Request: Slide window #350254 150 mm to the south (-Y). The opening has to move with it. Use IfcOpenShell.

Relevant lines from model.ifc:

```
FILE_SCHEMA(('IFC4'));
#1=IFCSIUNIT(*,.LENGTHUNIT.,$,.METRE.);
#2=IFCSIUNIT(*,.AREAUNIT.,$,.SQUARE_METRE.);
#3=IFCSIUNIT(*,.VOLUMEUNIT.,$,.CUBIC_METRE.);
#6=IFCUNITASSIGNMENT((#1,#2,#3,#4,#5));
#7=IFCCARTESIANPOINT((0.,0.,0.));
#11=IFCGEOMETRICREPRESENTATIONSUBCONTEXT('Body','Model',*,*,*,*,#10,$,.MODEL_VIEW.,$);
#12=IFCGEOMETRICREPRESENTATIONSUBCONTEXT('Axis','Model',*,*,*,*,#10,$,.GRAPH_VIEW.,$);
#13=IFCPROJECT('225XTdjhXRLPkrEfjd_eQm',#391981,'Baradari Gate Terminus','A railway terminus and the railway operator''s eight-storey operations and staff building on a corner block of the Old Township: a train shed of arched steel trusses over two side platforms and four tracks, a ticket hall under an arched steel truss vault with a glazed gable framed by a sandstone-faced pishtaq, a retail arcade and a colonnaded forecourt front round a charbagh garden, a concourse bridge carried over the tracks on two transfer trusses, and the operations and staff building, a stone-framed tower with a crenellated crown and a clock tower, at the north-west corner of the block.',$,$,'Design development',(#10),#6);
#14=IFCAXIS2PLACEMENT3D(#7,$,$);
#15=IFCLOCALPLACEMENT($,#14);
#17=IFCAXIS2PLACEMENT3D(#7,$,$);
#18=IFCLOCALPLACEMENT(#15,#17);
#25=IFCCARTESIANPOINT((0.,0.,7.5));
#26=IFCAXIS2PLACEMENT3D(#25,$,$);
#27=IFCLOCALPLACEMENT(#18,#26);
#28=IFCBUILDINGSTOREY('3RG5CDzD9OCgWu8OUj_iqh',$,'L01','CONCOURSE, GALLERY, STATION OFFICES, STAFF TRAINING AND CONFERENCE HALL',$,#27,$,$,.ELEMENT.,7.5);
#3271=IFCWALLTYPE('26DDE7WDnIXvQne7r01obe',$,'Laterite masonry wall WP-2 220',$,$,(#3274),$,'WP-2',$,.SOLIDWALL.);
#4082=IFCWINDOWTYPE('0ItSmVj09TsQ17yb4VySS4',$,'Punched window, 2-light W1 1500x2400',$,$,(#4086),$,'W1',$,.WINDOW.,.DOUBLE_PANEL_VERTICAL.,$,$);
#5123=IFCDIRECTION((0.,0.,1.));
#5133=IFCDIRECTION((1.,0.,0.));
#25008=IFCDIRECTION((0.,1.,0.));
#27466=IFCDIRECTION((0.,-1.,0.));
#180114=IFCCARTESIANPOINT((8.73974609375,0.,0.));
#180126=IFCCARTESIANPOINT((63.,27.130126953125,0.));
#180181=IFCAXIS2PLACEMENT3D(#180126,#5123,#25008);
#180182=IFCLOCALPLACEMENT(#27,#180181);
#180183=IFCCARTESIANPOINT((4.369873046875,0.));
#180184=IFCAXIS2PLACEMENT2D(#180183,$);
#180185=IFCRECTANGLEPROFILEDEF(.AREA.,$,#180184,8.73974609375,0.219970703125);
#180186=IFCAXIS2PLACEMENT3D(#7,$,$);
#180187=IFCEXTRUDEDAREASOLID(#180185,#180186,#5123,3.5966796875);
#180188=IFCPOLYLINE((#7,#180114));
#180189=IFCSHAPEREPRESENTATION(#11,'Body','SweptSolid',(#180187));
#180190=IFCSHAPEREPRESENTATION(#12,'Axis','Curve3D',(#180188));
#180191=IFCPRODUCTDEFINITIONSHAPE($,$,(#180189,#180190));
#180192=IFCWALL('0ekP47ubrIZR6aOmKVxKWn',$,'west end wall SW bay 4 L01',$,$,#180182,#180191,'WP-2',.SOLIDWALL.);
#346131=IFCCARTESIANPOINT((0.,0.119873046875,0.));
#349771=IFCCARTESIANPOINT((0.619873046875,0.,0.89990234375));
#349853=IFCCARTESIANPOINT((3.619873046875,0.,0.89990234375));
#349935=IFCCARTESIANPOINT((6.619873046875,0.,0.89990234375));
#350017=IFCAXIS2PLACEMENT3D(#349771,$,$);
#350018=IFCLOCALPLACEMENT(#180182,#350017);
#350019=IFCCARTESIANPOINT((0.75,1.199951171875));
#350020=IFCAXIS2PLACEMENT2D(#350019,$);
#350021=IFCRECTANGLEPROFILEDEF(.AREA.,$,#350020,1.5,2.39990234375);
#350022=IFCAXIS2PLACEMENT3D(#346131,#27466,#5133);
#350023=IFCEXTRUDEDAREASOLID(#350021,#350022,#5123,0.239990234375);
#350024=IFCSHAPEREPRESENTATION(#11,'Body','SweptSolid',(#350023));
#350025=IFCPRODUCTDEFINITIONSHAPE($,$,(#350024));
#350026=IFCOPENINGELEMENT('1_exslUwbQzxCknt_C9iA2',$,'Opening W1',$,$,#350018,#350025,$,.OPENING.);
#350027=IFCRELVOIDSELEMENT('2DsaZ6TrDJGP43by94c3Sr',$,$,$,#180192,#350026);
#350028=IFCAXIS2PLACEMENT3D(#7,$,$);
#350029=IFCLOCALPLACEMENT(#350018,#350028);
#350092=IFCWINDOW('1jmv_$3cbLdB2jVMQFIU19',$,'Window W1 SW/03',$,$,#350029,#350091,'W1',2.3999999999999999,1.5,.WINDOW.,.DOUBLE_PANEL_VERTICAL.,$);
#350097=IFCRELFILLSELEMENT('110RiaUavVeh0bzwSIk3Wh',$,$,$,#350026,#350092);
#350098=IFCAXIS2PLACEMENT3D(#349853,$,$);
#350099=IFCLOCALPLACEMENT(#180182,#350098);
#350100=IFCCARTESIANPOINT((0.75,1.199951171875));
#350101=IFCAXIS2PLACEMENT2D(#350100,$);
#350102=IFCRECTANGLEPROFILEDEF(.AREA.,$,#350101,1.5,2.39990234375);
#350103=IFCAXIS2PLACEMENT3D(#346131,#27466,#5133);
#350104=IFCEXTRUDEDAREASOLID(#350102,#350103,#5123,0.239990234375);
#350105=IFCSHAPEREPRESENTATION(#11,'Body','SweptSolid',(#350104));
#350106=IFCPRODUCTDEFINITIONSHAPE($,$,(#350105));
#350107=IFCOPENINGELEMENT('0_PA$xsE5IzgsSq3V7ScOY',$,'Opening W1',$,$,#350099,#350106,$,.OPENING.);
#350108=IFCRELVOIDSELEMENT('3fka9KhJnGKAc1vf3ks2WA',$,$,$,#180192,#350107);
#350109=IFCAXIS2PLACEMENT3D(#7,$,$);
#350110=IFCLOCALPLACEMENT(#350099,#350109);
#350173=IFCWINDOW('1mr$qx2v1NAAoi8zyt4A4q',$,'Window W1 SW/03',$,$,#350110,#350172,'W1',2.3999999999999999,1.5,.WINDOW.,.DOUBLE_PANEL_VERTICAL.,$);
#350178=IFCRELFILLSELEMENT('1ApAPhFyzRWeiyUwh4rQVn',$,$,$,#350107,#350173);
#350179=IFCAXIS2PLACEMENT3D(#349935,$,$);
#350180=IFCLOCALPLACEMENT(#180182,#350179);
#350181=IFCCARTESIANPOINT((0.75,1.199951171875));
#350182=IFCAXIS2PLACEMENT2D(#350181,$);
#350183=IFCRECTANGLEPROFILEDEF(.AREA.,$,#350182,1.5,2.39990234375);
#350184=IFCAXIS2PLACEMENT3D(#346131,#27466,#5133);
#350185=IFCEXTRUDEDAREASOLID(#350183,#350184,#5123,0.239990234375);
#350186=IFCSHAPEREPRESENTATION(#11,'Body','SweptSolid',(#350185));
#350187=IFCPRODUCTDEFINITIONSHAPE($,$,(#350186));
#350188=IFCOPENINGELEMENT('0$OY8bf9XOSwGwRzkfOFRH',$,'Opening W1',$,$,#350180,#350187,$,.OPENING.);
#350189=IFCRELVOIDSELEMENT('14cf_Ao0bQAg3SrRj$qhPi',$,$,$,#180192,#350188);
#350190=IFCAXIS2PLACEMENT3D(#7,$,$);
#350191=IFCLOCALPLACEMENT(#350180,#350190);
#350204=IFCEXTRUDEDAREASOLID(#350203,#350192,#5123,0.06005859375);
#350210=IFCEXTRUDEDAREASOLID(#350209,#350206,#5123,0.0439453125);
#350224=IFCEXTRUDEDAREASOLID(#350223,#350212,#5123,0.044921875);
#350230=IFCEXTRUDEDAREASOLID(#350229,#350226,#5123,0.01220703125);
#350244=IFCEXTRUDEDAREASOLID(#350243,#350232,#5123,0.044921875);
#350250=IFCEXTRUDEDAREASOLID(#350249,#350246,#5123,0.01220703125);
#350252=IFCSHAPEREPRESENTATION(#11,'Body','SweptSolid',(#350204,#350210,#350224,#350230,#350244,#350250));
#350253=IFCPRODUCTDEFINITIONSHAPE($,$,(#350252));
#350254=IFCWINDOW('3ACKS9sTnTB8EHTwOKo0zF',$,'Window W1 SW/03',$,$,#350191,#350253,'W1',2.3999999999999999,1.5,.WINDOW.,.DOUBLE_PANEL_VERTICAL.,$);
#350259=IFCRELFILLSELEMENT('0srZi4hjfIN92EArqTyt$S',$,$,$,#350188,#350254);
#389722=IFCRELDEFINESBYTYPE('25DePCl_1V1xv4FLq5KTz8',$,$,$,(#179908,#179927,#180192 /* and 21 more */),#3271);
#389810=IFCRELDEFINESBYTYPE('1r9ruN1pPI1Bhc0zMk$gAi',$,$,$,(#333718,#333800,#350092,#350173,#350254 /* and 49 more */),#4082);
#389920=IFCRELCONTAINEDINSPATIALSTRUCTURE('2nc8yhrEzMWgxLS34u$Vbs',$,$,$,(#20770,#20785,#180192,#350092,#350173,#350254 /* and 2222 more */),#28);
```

```python
import ifcopenshell
import ifcopenshell.api.geometry
import ifcopenshell.util.placement

model = ifcopenshell.open("model.ifc")

window = model.by_guid("3ACKS9sTnTB8EHTwOKo0zF")
opening = window.FillsVoids[0].RelatingOpeningElement
wall = opening.VoidsElements[0].RelatingBuildingElement

wall_matrix = ifcopenshell.util.placement.get_local_placement(wall.ObjectPlacement)
shift = wall_matrix[:3, 0] * -0.15
before = ifcopenshell.util.placement.get_local_placement(window.ObjectPlacement)[:3, 3].copy()

# The window is placed relative to its opening, so it follows when the opening moves.
matrix = ifcopenshell.util.placement.get_local_placement(opening.ObjectPlacement)
matrix[:3, 3] += shift
ifcopenshell.api.geometry.edit_object_placement(
    model, product=opening, matrix=matrix, is_si=False, should_transform_children=True
)

after = ifcopenshell.util.placement.get_local_placement(window.ObjectPlacement)[:3, 3]
print("window moved by", (after - before).round(3) + 0.0)

model.write("model_updated.ifc")
```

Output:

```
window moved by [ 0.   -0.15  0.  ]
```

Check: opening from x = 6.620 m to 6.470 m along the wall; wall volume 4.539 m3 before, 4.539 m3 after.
